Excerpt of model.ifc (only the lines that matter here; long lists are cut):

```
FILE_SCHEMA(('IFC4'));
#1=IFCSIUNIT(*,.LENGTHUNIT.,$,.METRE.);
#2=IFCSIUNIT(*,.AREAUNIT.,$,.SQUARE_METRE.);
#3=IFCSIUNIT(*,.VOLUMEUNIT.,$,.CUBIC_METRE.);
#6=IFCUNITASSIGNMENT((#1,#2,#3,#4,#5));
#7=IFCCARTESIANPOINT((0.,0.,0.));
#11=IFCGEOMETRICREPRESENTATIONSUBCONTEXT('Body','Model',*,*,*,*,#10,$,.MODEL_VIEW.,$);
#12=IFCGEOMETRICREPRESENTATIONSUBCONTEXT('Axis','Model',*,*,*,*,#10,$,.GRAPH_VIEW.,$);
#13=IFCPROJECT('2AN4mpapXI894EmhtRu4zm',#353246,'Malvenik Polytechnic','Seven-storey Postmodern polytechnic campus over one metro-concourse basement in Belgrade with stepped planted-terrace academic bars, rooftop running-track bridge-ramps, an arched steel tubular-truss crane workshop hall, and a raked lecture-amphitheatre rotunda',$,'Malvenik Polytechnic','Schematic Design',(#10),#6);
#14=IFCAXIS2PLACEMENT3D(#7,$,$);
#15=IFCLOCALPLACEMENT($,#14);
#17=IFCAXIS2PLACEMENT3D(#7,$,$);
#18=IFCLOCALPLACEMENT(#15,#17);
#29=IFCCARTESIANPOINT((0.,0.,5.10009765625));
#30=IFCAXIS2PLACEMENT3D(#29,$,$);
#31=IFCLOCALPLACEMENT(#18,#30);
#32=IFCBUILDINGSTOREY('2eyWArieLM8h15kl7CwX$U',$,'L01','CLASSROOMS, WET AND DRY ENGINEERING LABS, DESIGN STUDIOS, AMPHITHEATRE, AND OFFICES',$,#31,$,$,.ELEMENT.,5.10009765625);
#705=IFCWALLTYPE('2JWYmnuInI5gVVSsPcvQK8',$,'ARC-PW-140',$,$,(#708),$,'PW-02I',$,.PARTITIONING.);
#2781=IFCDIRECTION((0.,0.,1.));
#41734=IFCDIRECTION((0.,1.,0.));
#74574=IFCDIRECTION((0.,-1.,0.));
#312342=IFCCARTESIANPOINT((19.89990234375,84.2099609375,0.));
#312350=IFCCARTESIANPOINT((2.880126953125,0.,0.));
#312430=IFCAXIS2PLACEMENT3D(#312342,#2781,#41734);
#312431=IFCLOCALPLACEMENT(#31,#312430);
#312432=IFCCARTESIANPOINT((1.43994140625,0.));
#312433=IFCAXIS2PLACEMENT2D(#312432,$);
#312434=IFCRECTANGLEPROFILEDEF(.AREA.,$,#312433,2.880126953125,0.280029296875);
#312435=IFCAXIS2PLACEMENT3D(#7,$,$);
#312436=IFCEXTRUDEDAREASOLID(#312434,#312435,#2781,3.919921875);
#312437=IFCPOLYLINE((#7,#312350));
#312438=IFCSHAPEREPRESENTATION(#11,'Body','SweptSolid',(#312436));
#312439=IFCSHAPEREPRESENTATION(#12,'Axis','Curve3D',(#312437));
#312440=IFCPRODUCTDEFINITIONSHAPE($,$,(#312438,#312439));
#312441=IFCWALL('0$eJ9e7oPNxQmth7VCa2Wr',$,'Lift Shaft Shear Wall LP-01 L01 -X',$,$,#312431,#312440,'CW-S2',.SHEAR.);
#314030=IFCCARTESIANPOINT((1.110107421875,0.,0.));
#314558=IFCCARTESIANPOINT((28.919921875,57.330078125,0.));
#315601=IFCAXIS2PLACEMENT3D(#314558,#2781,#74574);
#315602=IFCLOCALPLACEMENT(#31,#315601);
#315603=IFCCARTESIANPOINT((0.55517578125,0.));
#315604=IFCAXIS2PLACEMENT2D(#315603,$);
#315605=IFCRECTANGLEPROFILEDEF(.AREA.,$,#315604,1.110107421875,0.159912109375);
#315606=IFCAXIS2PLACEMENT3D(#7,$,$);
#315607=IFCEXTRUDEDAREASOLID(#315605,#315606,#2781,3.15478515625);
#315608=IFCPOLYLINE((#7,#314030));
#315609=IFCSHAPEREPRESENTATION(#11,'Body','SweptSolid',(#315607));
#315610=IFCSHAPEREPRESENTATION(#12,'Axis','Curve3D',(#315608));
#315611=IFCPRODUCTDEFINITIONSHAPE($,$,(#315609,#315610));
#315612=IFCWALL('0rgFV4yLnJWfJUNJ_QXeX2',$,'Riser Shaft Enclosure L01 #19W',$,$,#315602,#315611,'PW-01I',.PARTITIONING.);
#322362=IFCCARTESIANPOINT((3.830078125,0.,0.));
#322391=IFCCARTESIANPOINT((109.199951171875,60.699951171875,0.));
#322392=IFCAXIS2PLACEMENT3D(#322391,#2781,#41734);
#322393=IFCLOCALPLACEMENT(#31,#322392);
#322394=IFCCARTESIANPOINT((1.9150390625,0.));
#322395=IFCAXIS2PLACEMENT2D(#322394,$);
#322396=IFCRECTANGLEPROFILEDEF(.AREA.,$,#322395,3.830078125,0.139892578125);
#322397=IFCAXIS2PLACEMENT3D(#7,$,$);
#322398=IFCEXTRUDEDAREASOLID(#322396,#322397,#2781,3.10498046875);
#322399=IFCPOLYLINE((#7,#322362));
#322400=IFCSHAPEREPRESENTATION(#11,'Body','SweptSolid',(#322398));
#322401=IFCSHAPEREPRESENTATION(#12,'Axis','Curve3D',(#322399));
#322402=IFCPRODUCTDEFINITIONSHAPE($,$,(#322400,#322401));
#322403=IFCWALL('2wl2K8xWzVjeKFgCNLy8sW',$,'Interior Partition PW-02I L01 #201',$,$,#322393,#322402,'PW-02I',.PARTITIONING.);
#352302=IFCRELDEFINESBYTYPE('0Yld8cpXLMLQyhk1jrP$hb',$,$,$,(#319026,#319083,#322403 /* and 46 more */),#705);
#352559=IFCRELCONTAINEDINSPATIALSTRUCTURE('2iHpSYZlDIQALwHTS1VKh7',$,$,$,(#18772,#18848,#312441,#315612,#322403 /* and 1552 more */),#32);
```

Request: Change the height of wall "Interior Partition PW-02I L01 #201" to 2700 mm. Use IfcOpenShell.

```python
import ifcopenshell
import ifcopenshell.geom
import ifcopenshell.util.representation
import ifcopenshell.util.shape
import ifcopenshell.util.unit

model = ifcopenshell.open("model.ifc")
unit_scale = ifcopenshell.util.unit.calculate_unit_scale(model)
settings = ifcopenshell.geom.settings()


def volume(element):
    """Net volume in cubic metres, openings subtracted."""
    shape = ifcopenshell.geom.create_shape(settings, element)
    return ifcopenshell.util.shape.get_volume(shape.geometry)


wall = model.by_guid("2wl2K8xWzVjeKFgCNLy8sW")
before = volume(wall)

body = ifcopenshell.util.representation.get_representation(wall, "Model", "Body")
solid = body.Items[0]
old_height = solid.Depth
solid.Depth = 2.7 / unit_scale
after = volume(wall)

print(f"height {old_height:g} -> {solid.Depth:g}, volume {before:.3f} -> {after:.3f} m3")

model.write("model-out.ifc")
```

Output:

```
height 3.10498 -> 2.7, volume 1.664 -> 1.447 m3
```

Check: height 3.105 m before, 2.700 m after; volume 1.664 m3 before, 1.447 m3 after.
